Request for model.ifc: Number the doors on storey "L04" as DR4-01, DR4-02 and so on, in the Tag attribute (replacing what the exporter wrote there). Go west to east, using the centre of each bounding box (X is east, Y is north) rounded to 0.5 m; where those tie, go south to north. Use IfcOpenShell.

First a look at what the model holds.

```python
import ifcopenshell
import ifcopenshell.util.element
import ifcopenshell.util.placement

model = ifcopenshell.open("model.ifc")
print(model.schema)
storey = next(s for s in model.by_type("IfcBuildingStorey") if s.Name == "L04")
doors = [e for e in ifcopenshell.util.element.get_decomposition(storey) if e.is_a("IfcDoor")]
for e in sorted(doors, key=lambda e: e.id()):
    origin = ifcopenshell.util.placement.get_local_placement(e.ObjectPlacement)[:3, 3]
    print(e.id(), e.Tag, e.Name, origin.round(2) + 0.0, sep=" | ")
```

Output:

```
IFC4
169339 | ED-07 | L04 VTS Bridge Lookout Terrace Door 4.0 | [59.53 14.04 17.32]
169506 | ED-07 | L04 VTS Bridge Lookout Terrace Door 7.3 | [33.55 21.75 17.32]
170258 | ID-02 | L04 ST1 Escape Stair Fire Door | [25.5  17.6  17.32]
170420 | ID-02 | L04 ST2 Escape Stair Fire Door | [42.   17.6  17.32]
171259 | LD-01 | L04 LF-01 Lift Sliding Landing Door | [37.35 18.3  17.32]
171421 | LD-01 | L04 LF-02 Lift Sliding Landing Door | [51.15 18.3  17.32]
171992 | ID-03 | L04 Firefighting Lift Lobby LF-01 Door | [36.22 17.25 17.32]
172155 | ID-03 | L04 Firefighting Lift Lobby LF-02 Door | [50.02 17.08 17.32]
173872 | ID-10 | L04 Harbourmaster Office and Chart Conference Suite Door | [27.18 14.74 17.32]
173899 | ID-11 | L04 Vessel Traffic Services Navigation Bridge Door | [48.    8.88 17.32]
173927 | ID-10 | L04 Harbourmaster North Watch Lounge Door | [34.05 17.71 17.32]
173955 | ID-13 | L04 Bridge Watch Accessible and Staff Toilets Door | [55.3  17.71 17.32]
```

```python
import ifcopenshell
import ifcopenshell.geom
import ifcopenshell.util.element
import ifcopenshell.util.shape

model = ifcopenshell.open("model.ifc")
settings = ifcopenshell.geom.settings()
settings.set("use-world-coords", True)


def centre(element):
    shape = ifcopenshell.geom.create_shape(settings, element)
    return ifcopenshell.util.shape.get_bbox_centroid(shape.geometry)


storey = next(s for s in model.by_type("IfcBuildingStorey") if s.Name == "L04")
doors = [e for e in ifcopenshell.util.element.get_decomposition(storey) if e.is_a("IfcDoor")]

# Insertion points can sit at a corner or the storey origin, so sort by the geometry (in metres).
centres = {e: centre(e) for e in doors}
doors.sort(key=lambda e: (round(centres[e][0] / 0.5), centres[e][1]))

for i, e in enumerate(doors, start=1):
    number = f"DR4-{i:02d}"
    e.Tag = number
    print(e.id(), number)

model.write("model_rev.ifc")
```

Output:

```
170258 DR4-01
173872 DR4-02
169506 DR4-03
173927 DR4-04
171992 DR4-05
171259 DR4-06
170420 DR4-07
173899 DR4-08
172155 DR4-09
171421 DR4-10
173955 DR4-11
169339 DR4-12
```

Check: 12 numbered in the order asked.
